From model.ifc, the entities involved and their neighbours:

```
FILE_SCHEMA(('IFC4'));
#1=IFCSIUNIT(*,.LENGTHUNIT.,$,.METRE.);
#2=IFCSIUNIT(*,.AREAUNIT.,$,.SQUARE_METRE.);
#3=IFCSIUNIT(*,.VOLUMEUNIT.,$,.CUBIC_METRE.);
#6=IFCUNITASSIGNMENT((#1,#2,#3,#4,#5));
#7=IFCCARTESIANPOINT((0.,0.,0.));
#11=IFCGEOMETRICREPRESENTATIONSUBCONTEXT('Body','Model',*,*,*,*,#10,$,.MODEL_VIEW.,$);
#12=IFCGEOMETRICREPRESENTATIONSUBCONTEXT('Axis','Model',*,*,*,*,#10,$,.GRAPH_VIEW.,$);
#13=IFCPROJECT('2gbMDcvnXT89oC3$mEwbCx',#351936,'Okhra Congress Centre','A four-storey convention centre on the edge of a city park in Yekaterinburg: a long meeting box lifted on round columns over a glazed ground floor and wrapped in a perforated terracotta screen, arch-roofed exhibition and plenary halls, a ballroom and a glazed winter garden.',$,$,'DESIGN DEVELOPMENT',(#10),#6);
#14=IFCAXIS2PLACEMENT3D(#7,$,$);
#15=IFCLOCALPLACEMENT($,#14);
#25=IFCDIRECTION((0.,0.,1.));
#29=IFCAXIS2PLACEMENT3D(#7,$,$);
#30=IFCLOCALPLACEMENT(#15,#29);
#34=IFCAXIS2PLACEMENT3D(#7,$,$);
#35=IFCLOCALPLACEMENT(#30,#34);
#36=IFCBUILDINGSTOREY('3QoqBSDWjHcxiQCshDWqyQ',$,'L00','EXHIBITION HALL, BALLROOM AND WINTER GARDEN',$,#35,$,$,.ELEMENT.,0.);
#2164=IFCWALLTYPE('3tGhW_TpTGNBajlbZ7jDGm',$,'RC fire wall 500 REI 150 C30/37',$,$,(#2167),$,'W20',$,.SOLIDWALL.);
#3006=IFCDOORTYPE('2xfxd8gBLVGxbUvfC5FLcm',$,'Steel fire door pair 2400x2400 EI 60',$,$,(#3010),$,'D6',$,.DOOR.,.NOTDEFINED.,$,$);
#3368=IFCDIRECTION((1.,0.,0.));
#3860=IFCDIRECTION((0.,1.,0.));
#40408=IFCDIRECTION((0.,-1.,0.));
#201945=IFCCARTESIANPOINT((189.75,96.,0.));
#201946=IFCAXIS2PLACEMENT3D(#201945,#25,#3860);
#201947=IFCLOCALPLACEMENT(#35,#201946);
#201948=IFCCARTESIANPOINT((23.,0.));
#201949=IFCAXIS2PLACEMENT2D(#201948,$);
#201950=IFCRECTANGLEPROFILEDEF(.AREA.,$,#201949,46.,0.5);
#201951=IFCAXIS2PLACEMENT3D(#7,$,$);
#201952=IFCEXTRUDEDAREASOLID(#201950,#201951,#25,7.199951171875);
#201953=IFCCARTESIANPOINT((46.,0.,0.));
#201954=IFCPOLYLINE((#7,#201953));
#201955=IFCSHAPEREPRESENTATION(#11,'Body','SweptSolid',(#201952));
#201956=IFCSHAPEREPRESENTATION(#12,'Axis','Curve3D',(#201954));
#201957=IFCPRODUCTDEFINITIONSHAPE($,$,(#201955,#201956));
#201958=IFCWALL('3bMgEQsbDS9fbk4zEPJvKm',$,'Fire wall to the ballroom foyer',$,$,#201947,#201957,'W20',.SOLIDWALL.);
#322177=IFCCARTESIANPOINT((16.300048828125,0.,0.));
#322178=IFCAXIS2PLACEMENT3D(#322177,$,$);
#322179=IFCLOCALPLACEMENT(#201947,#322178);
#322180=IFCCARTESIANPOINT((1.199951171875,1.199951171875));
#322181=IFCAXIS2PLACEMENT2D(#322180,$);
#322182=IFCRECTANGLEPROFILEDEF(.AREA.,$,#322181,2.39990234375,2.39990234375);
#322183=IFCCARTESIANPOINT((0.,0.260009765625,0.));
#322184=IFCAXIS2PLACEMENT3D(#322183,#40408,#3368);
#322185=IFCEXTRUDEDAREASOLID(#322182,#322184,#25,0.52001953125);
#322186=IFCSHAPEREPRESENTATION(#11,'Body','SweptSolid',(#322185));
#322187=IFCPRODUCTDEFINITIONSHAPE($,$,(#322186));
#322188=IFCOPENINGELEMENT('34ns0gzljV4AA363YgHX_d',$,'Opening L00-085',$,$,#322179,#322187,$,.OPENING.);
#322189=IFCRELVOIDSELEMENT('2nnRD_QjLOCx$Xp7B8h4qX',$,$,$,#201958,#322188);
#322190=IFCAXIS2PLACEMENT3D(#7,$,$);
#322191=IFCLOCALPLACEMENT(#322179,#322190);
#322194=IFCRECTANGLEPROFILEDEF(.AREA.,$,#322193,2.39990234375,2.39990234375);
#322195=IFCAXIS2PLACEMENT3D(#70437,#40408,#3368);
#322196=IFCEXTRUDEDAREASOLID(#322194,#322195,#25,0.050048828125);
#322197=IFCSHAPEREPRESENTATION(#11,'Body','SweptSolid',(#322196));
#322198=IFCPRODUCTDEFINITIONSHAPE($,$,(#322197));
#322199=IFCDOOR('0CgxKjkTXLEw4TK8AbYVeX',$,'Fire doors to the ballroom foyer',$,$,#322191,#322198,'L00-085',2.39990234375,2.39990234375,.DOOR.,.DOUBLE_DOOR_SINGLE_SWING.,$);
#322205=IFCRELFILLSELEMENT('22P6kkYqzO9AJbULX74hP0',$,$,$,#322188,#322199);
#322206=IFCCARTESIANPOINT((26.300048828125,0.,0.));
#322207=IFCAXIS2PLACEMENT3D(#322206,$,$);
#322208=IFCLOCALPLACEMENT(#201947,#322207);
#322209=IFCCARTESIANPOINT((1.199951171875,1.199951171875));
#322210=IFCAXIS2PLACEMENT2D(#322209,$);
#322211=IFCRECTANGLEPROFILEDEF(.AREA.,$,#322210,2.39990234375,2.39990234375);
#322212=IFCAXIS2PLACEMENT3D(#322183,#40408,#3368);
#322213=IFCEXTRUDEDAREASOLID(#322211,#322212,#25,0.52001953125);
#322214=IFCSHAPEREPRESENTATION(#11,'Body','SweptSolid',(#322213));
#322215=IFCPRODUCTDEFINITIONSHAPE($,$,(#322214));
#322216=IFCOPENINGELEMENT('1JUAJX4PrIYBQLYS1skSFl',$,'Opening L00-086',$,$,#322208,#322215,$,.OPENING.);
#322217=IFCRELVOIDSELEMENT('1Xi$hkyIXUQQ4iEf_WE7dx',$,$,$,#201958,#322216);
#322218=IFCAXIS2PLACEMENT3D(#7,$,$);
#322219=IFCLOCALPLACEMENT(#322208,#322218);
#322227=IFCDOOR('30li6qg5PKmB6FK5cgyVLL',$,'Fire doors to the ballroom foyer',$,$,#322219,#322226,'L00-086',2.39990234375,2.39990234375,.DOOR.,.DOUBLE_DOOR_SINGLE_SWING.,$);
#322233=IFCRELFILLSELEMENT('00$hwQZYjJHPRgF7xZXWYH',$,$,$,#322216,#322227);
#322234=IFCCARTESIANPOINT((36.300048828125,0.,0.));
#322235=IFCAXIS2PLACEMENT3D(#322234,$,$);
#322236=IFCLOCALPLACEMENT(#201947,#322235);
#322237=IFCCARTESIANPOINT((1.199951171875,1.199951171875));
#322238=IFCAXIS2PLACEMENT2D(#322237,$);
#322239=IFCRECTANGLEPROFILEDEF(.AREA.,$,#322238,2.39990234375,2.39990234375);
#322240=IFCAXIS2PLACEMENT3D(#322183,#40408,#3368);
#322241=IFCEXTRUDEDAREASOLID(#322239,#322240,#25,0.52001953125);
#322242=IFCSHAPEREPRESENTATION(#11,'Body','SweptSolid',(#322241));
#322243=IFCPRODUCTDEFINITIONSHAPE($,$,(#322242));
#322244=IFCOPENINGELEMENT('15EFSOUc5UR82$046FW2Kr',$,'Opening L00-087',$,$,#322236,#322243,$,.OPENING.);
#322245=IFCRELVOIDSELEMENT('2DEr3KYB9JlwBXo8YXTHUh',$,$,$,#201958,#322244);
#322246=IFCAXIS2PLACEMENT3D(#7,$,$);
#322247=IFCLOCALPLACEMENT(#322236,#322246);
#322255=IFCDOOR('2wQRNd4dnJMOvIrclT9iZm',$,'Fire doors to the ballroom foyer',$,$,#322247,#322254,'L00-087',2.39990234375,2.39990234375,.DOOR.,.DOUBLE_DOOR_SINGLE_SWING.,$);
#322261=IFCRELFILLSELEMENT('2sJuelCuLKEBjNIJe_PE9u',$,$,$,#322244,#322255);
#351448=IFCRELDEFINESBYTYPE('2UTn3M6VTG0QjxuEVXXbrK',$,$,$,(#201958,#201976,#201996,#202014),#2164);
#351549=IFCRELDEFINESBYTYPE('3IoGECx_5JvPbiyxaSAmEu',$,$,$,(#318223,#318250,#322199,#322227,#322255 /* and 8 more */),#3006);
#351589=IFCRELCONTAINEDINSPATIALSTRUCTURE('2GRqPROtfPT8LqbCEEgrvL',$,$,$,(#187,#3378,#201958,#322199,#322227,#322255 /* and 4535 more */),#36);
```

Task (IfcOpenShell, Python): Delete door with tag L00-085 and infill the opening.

```python
import ifcopenshell
import ifcopenshell.api.feature
import ifcopenshell.api.root
import ifcopenshell.geom
import ifcopenshell.util.shape

model = ifcopenshell.open("model.ifc")
settings = ifcopenshell.geom.settings()


def volume(element):
    """Net volume in cubic metres, openings subtracted."""
    shape = ifcopenshell.geom.create_shape(settings, element)
    return ifcopenshell.util.shape.get_volume(shape.geometry)


door = model.by_id(322199)
opening = door.FillsVoids[0].RelatingOpeningElement
wall = opening.VoidsElements[0].RelatingBuildingElement
before = volume(wall)

ifcopenshell.api.root.remove_product(model, product=door)
ifcopenshell.api.feature.remove_feature(model, feature=opening)

after = volume(wall)

print(f"wall volume {before:.3f} -> {after:.3f} m3")

model.write("model_v2.ifc")
```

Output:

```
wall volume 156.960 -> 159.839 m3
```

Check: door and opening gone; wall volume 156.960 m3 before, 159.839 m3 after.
